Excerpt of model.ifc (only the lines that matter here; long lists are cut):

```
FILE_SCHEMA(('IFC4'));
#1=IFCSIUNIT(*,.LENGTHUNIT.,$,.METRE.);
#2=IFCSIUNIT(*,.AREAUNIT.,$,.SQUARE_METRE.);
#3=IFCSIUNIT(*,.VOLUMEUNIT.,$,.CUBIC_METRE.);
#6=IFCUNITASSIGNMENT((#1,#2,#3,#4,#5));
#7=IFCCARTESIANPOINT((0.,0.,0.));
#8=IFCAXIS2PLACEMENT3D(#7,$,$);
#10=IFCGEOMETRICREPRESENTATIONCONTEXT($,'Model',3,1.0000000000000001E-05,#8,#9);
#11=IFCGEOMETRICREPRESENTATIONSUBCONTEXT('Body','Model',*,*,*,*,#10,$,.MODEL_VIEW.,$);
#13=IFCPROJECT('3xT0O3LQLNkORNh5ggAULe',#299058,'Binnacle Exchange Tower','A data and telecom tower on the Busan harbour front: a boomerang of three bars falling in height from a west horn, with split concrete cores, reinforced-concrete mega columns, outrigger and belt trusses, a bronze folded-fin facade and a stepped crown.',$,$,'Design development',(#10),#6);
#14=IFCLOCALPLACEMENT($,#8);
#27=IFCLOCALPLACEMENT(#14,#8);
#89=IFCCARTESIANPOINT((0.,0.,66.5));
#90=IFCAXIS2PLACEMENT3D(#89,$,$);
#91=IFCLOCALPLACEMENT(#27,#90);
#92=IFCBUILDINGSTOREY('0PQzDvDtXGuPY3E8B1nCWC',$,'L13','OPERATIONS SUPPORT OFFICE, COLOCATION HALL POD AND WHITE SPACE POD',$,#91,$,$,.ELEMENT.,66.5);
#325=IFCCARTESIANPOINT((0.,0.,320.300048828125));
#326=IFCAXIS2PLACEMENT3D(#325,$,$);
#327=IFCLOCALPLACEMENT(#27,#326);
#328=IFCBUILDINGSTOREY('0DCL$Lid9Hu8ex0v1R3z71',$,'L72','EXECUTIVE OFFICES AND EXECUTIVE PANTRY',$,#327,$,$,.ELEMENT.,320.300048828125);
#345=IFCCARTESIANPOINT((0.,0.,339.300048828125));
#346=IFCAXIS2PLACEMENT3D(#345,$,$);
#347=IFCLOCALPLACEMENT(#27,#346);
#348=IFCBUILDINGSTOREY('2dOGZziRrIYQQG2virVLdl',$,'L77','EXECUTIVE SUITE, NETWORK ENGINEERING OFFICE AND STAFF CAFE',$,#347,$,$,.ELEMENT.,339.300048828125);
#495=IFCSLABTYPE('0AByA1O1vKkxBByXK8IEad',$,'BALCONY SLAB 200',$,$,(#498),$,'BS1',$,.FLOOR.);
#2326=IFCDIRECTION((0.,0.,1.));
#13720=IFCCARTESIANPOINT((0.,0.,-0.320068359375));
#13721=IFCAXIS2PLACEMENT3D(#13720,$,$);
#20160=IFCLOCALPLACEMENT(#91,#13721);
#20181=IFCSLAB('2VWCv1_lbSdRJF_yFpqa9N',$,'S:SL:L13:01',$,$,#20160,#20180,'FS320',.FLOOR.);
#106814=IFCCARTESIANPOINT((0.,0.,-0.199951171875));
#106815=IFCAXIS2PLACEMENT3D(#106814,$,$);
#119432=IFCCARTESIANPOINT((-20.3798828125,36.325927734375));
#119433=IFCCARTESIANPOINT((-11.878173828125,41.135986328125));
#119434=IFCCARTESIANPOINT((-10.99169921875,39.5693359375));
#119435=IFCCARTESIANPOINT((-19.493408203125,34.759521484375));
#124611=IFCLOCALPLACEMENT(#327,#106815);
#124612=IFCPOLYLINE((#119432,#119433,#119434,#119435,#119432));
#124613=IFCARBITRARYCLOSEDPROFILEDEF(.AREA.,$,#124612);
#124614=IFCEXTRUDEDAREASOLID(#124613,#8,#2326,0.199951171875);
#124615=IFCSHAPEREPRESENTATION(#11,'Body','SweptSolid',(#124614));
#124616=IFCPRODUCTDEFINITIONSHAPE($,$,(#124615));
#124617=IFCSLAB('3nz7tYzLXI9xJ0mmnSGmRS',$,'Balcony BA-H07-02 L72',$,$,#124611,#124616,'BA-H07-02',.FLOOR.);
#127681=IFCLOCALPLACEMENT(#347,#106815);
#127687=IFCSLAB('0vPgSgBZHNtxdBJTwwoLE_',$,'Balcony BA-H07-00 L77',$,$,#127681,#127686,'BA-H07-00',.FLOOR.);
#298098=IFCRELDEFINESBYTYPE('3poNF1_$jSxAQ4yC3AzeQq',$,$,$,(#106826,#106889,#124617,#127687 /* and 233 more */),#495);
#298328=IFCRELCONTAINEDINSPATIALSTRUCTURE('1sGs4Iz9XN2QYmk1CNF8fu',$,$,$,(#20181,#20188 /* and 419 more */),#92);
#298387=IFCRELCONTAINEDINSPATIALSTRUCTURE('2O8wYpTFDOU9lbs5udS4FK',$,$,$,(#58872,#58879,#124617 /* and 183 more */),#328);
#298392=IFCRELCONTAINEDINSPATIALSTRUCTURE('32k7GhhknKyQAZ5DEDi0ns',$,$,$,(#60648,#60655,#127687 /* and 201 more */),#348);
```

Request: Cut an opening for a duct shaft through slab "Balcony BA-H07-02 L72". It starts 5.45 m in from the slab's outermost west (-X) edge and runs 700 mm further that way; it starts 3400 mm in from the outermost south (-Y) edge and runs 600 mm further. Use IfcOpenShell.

```python
import numpy as np
import ifcopenshell
import ifcopenshell.api.feature
import ifcopenshell.api.geometry
import ifcopenshell.api.root
import ifcopenshell.geom
import ifcopenshell.util.placement
import ifcopenshell.util.representation
import ifcopenshell.util.shape
import ifcopenshell.util.unit

model = ifcopenshell.open("model.ifc")
unit_scale = ifcopenshell.util.unit.calculate_unit_scale(model)
settings = ifcopenshell.geom.settings()


def volume(element):
    """Net volume in cubic metres, openings subtracted."""
    shape = ifcopenshell.geom.create_shape(settings, element)
    return ifcopenshell.util.shape.get_volume(shape.geometry)


slab = model.by_guid("3nz7tYzLXI9xJ0mmnSGmRS")
before = volume(slab)

# Extent in the slab's own axes, in metres. The edges named are its -X and -Y sides.
slab_shape = ifcopenshell.geom.create_shape(settings, slab)
vertices = ifcopenshell.util.shape.get_vertices(slab_shape.geometry)
x_min, y_min, bottom = vertices.min(axis=0)
top = vertices[:, 2].max()

opening = ifcopenshell.api.root.create_entity(model, ifc_class="IfcOpeningElement", name="Duct shaft opening", predefined_type="OPENING")
context = ifcopenshell.util.representation.get_context(model, "Model", "Body", "MODEL_VIEW")
width, depth = 0.7, 0.6
outline = [(0.0, 0.0), (width, 0.0), (width, depth), (0.0, depth), (0.0, 0.0)]
# Overshoot both faces by 50 mm so the cut is clean.
shape = ifcopenshell.api.geometry.add_slab_representation(
    model, context=context, depth=top - bottom + 0.1, polyline=outline
)
ifcopenshell.api.geometry.assign_representation(model, product=opening, representation=shape)

matrix = ifcopenshell.util.placement.get_local_placement(slab.ObjectPlacement)
matrix[:, 3] = matrix @ np.append(np.array([x_min + 5.45, y_min + 3.4, bottom - 0.05]) / unit_scale, 1.0)
ifcopenshell.api.geometry.edit_object_placement(model, product=opening, matrix=matrix, is_si=False)
ifcopenshell.api.feature.add_feature(model, feature=opening, element=slab)

after = volume(slab)

print(f"slab volume {before:.3f} -> {after:.3f} m3")

model.write("model-out.ifc")
```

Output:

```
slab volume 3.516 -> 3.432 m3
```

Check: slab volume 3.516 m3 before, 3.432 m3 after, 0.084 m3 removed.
